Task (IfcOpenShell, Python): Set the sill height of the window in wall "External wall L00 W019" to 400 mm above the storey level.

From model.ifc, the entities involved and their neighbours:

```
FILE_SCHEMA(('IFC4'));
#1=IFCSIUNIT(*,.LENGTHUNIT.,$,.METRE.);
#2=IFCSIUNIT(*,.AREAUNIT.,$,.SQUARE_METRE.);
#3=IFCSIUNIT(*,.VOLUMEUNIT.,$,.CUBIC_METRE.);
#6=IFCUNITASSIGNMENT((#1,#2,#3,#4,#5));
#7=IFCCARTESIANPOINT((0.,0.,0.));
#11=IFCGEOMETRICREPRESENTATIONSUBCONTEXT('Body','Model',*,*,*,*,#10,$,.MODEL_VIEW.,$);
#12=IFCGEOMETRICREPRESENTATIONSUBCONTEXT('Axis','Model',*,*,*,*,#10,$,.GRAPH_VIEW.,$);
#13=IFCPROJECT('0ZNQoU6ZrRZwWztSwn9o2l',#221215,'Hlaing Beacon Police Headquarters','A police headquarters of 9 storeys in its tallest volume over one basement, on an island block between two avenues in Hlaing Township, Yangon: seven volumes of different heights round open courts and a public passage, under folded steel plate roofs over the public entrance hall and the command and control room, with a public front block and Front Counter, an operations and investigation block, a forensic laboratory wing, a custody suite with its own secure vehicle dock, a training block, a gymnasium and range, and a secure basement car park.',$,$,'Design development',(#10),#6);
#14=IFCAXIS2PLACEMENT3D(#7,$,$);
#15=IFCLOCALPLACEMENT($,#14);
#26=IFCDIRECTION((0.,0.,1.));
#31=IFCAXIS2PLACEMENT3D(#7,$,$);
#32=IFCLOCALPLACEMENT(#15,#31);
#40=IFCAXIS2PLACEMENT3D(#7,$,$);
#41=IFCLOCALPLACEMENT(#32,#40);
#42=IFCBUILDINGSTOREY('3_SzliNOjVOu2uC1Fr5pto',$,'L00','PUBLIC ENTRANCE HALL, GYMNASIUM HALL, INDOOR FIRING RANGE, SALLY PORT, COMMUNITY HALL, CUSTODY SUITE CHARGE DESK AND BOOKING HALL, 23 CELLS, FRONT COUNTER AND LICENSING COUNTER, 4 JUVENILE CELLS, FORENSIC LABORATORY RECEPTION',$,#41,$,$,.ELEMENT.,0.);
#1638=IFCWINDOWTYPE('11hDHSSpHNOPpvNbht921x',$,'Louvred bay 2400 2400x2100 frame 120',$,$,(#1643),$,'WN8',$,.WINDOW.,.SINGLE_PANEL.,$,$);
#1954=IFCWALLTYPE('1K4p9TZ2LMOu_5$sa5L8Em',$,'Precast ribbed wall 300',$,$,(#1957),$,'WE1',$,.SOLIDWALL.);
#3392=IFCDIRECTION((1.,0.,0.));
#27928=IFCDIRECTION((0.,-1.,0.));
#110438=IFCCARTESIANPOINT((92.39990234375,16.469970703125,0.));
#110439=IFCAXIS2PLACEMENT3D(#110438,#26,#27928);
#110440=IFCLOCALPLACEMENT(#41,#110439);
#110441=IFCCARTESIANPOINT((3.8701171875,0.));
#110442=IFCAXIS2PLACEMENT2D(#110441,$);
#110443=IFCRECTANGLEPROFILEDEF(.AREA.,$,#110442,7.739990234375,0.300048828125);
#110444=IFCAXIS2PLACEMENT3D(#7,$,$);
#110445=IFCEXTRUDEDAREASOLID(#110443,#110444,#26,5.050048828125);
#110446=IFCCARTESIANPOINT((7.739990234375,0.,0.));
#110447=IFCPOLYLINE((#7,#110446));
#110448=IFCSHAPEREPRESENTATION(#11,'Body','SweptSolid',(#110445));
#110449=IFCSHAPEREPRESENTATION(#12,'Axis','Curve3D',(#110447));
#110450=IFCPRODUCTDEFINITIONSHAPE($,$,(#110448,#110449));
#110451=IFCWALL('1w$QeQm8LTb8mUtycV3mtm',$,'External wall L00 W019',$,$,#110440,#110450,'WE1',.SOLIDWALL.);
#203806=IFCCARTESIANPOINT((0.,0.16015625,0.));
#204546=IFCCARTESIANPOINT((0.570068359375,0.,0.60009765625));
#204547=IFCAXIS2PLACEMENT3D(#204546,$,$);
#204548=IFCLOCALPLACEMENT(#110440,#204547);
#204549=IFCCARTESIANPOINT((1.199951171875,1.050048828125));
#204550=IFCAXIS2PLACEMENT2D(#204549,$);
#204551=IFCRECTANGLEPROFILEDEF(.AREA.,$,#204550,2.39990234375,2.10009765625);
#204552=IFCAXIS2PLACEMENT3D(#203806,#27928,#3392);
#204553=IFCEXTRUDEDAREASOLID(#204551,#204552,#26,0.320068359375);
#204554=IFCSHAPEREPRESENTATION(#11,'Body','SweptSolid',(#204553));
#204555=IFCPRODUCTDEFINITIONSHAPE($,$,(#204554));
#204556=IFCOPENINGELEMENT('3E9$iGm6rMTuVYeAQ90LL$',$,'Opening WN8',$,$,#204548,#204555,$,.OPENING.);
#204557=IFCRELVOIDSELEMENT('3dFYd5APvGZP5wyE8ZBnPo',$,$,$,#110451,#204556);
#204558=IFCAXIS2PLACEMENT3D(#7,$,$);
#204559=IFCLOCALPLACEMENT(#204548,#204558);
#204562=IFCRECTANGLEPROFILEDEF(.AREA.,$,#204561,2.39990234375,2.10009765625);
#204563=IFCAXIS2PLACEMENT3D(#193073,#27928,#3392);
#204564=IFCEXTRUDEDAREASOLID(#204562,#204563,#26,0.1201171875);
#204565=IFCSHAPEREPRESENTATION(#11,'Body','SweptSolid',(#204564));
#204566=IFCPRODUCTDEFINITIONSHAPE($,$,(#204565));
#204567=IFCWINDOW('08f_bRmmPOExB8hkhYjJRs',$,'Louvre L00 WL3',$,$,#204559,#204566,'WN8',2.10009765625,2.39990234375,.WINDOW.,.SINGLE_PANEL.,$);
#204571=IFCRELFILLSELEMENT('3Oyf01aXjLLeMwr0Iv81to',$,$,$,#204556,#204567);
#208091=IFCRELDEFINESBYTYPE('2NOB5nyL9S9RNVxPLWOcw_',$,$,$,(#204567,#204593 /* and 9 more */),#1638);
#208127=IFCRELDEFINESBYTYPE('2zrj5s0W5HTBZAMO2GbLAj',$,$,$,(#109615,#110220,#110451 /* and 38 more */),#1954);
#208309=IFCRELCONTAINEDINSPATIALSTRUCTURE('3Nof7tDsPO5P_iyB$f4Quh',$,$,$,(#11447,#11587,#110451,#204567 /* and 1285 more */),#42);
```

```python
import numpy as np
import ifcopenshell
import ifcopenshell.api.geometry
import ifcopenshell.geom
import ifcopenshell.util.element
import ifcopenshell.util.placement
import ifcopenshell.util.shape
import ifcopenshell.util.unit

model = ifcopenshell.open("model.ifc")
unit_scale = ifcopenshell.util.unit.calculate_unit_scale(model)

window = model.by_guid("08f_bRmmPOExB8hkhYjJRs")
opening = window.FillsVoids[0].RelatingOpeningElement
storey = ifcopenshell.util.element.get_container(window, ifc_class="IfcBuildingStorey")
level = ifcopenshell.util.placement.get_local_placement(storey.ObjectPlacement)[2, 3]

# The opening's origin need not be at the sill, so measure its lowest point.
shape = ifcopenshell.geom.create_shape(ifcopenshell.geom.settings(), opening)
bottom = ifcopenshell.util.shape.get_shape_bottom_elevation(shape, shape.geometry) / unit_scale
dz = level + 0.4 / unit_scale - bottom

shift = np.array([0.0, 0.0, dz])
# The window is placed relative to its opening, so it follows when the opening moves.
matrix = ifcopenshell.util.placement.get_local_placement(opening.ObjectPlacement)
matrix[:3, 3] += shift
ifcopenshell.api.geometry.edit_object_placement(
    model, product=opening, matrix=matrix, is_si=False, should_transform_children=True
)

print(f"moved by {dz * unit_scale:+.3f} m")

model.write("model_v2.ifc")
```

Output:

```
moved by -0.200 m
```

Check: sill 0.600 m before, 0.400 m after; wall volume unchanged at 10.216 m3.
